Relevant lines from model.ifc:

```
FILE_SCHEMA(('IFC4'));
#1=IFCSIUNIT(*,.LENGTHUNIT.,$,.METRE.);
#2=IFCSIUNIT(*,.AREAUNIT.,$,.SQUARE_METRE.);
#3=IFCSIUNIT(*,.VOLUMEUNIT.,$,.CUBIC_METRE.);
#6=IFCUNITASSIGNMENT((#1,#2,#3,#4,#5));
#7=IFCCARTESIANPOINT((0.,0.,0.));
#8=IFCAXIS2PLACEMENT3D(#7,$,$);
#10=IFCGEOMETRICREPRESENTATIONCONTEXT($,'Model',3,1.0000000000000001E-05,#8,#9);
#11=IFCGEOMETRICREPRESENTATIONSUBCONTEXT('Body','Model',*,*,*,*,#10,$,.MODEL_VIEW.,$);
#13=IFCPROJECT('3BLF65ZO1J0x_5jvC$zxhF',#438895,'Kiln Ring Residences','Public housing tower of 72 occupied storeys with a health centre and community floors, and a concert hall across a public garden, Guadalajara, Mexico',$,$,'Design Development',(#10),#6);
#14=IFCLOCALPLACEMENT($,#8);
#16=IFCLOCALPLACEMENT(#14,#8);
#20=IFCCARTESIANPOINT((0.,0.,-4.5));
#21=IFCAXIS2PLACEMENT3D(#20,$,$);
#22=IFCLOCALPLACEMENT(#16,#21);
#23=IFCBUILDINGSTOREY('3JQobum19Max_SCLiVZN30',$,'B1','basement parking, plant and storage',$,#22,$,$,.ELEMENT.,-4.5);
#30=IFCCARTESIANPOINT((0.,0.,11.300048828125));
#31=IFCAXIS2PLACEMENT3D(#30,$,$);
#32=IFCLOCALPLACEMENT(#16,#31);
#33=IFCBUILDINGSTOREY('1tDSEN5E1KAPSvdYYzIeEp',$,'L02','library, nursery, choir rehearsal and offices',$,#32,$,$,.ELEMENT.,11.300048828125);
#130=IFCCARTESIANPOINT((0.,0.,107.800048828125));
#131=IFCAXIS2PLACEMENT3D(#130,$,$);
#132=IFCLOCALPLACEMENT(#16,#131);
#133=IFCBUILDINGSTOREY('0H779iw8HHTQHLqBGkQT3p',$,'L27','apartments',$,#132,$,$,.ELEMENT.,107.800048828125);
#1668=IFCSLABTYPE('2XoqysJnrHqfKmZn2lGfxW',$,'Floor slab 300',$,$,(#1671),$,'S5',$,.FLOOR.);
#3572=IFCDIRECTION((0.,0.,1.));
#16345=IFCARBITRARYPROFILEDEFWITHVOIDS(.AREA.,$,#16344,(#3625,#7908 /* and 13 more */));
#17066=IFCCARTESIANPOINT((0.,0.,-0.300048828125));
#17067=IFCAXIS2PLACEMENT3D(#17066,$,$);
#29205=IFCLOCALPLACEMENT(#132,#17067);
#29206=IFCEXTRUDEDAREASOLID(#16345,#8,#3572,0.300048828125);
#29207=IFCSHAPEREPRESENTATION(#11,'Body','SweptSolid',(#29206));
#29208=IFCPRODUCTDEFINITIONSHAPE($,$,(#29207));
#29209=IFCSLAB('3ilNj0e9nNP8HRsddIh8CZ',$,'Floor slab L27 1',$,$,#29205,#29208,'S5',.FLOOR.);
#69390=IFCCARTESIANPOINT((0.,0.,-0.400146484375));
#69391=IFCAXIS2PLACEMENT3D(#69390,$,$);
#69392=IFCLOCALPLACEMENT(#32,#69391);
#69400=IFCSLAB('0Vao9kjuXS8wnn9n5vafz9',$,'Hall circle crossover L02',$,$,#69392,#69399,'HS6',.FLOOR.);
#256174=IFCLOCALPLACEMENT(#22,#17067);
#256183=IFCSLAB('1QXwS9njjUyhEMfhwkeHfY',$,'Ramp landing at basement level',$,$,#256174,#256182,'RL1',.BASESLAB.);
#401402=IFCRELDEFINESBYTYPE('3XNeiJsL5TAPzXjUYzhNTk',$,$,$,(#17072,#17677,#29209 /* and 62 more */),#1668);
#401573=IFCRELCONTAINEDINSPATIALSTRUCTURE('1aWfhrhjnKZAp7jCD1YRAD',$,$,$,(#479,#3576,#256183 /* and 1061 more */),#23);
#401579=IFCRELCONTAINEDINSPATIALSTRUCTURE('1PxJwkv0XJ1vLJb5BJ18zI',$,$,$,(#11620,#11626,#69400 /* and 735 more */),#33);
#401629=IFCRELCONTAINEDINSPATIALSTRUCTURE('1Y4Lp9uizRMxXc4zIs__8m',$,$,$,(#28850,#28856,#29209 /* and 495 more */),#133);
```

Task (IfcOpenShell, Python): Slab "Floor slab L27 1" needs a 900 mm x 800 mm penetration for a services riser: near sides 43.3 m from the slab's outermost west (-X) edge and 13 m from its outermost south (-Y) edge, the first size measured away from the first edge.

```python
import numpy as np
import ifcopenshell
import ifcopenshell.api.feature
import ifcopenshell.api.geometry
import ifcopenshell.api.root
import ifcopenshell.geom
import ifcopenshell.util.placement
import ifcopenshell.util.representation
import ifcopenshell.util.shape
import ifcopenshell.util.unit

model = ifcopenshell.open("model.ifc")
unit_scale = ifcopenshell.util.unit.calculate_unit_scale(model)
settings = ifcopenshell.geom.settings()


def volume(element):
    """Net volume in cubic metres, openings subtracted."""
    shape = ifcopenshell.geom.create_shape(settings, element)
    return ifcopenshell.util.shape.get_volume(shape.geometry)


slab = model.by_guid("3ilNj0e9nNP8HRsddIh8CZ")
before = volume(slab)

# Extent in the slab's own axes, in metres. The edges named are its -X and -Y sides.
slab_shape = ifcopenshell.geom.create_shape(settings, slab)
vertices = ifcopenshell.util.shape.get_vertices(slab_shape.geometry)
x_min, y_min, bottom = vertices.min(axis=0)
top = vertices[:, 2].max()

opening = ifcopenshell.api.root.create_entity(model, ifc_class="IfcOpeningElement", name="Services riser opening", predefined_type="OPENING")
context = ifcopenshell.util.representation.get_context(model, "Model", "Body", "MODEL_VIEW")
width, depth = 0.9, 0.8
outline = [(0.0, 0.0), (width, 0.0), (width, depth), (0.0, depth), (0.0, 0.0)]
# Overshoot both faces by 50 mm so the cut is clean.
shape = ifcopenshell.api.geometry.add_slab_representation(
    model, context=context, depth=top - bottom + 0.1, polyline=outline
)
ifcopenshell.api.geometry.assign_representation(model, product=opening, representation=shape)

matrix = ifcopenshell.util.placement.get_local_placement(slab.ObjectPlacement)
matrix[:, 3] = matrix @ np.append(np.array([x_min + 43.3, y_min + 13, bottom - 0.05]) / unit_scale, 1.0)
ifcopenshell.api.geometry.edit_object_placement(model, product=opening, matrix=matrix, is_si=False)
ifcopenshell.api.feature.add_feature(model, feature=opening, element=slab)

after = volume(slab)

print(f"slab volume {before:.3f} -> {after:.3f} m3")

model.write("model_rev.ifc")
```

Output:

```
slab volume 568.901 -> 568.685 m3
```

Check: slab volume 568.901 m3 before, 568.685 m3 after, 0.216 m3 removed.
